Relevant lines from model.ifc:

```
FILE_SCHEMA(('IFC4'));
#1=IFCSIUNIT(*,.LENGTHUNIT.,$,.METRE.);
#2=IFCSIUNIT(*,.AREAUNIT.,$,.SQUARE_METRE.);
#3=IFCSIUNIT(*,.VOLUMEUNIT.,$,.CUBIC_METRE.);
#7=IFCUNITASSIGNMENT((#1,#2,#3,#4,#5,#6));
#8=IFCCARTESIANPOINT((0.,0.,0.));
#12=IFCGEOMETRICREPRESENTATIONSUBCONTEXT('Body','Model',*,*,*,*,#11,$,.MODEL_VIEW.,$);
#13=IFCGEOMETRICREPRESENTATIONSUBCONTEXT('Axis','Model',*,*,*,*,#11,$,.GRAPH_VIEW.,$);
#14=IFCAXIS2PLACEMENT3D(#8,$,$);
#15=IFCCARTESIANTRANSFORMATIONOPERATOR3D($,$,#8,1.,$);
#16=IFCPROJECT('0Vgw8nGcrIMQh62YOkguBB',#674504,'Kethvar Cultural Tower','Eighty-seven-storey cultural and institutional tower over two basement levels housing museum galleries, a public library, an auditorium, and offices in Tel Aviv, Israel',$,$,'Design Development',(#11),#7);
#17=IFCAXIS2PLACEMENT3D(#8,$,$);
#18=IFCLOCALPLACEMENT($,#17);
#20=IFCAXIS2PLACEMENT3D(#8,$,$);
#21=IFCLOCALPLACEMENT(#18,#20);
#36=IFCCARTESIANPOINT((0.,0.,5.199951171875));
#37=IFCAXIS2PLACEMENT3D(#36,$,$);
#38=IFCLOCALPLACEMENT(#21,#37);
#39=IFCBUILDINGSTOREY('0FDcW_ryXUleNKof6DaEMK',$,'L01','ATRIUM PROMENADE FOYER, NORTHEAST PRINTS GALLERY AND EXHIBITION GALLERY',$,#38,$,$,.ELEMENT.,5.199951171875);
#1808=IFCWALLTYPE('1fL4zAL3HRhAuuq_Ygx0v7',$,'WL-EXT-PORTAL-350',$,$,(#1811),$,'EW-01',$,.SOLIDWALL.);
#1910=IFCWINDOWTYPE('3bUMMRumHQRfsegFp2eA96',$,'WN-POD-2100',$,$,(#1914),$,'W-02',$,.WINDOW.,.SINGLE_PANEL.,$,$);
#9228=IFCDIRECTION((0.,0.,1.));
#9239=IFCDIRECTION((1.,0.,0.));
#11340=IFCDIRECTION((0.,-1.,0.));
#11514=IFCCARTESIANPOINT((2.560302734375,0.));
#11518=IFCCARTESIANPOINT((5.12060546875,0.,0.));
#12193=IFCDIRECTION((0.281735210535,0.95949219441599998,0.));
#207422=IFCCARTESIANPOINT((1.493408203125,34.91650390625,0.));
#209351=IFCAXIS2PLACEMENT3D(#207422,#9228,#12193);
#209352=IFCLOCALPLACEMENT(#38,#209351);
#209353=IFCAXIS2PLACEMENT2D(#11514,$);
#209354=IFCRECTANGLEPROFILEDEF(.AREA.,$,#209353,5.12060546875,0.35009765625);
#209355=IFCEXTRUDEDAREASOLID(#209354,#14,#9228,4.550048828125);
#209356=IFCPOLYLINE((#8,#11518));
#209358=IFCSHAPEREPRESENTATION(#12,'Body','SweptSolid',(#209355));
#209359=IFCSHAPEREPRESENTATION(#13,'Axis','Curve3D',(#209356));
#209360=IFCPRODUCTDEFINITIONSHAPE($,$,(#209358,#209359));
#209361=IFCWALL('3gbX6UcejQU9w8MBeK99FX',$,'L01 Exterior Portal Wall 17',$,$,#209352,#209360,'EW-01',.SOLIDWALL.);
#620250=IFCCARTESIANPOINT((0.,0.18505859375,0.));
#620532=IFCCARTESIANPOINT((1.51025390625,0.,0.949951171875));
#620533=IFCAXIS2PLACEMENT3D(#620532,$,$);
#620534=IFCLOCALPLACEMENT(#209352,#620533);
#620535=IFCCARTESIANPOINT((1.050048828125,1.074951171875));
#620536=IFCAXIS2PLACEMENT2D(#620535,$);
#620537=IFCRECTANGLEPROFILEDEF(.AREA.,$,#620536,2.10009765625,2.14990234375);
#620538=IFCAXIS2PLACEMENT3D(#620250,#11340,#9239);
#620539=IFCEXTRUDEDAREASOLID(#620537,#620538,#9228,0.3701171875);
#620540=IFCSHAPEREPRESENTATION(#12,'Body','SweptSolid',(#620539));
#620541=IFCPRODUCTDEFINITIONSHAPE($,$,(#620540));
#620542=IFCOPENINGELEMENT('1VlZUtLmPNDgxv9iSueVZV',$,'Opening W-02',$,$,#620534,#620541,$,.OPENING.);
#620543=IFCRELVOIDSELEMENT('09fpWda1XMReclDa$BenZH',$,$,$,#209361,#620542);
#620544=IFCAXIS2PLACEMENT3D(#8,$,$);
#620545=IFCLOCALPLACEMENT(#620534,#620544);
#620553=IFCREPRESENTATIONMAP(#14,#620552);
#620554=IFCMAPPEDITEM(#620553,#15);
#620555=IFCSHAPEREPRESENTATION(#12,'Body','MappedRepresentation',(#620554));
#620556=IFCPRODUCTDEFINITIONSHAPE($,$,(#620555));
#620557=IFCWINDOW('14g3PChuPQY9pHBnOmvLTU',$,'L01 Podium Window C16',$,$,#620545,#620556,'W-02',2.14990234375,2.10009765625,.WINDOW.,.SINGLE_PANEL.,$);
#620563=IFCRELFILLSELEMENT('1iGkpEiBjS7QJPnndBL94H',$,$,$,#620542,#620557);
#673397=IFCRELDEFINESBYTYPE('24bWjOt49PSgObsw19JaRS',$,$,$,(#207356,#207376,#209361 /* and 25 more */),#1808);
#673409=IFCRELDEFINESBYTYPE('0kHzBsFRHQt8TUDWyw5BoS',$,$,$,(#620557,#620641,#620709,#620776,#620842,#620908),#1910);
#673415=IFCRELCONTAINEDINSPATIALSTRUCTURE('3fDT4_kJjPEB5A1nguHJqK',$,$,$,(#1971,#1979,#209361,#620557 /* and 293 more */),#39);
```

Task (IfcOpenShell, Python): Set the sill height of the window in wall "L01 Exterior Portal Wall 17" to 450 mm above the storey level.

```python
import numpy as np
import ifcopenshell
import ifcopenshell.api.geometry
import ifcopenshell.geom
import ifcopenshell.util.element
import ifcopenshell.util.placement
import ifcopenshell.util.shape
import ifcopenshell.util.unit

model = ifcopenshell.open("model.ifc")
unit_scale = ifcopenshell.util.unit.calculate_unit_scale(model)

window = model.by_guid("14g3PChuPQY9pHBnOmvLTU")
opening = window.FillsVoids[0].RelatingOpeningElement
storey = ifcopenshell.util.element.get_container(window, ifc_class="IfcBuildingStorey")
level = ifcopenshell.util.placement.get_local_placement(storey.ObjectPlacement)[2, 3]

# The opening's origin need not be at the sill, so measure its lowest point.
shape = ifcopenshell.geom.create_shape(ifcopenshell.geom.settings(), opening)
bottom = ifcopenshell.util.shape.get_shape_bottom_elevation(shape, shape.geometry) / unit_scale
dz = level + 0.45 / unit_scale - bottom

shift = np.array([0.0, 0.0, dz])
# The window is placed relative to its opening, so it follows when the opening moves.
matrix = ifcopenshell.util.placement.get_local_placement(opening.ObjectPlacement)
matrix[:3, 3] += shift
ifcopenshell.api.geometry.edit_object_placement(
    model, product=opening, matrix=matrix, is_si=False, should_transform_children=True
)

print(f"moved by {dz * unit_scale:+.3f} m")

model.write("model_rev.ifc")
```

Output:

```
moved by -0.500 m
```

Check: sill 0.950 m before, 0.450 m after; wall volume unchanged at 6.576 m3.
